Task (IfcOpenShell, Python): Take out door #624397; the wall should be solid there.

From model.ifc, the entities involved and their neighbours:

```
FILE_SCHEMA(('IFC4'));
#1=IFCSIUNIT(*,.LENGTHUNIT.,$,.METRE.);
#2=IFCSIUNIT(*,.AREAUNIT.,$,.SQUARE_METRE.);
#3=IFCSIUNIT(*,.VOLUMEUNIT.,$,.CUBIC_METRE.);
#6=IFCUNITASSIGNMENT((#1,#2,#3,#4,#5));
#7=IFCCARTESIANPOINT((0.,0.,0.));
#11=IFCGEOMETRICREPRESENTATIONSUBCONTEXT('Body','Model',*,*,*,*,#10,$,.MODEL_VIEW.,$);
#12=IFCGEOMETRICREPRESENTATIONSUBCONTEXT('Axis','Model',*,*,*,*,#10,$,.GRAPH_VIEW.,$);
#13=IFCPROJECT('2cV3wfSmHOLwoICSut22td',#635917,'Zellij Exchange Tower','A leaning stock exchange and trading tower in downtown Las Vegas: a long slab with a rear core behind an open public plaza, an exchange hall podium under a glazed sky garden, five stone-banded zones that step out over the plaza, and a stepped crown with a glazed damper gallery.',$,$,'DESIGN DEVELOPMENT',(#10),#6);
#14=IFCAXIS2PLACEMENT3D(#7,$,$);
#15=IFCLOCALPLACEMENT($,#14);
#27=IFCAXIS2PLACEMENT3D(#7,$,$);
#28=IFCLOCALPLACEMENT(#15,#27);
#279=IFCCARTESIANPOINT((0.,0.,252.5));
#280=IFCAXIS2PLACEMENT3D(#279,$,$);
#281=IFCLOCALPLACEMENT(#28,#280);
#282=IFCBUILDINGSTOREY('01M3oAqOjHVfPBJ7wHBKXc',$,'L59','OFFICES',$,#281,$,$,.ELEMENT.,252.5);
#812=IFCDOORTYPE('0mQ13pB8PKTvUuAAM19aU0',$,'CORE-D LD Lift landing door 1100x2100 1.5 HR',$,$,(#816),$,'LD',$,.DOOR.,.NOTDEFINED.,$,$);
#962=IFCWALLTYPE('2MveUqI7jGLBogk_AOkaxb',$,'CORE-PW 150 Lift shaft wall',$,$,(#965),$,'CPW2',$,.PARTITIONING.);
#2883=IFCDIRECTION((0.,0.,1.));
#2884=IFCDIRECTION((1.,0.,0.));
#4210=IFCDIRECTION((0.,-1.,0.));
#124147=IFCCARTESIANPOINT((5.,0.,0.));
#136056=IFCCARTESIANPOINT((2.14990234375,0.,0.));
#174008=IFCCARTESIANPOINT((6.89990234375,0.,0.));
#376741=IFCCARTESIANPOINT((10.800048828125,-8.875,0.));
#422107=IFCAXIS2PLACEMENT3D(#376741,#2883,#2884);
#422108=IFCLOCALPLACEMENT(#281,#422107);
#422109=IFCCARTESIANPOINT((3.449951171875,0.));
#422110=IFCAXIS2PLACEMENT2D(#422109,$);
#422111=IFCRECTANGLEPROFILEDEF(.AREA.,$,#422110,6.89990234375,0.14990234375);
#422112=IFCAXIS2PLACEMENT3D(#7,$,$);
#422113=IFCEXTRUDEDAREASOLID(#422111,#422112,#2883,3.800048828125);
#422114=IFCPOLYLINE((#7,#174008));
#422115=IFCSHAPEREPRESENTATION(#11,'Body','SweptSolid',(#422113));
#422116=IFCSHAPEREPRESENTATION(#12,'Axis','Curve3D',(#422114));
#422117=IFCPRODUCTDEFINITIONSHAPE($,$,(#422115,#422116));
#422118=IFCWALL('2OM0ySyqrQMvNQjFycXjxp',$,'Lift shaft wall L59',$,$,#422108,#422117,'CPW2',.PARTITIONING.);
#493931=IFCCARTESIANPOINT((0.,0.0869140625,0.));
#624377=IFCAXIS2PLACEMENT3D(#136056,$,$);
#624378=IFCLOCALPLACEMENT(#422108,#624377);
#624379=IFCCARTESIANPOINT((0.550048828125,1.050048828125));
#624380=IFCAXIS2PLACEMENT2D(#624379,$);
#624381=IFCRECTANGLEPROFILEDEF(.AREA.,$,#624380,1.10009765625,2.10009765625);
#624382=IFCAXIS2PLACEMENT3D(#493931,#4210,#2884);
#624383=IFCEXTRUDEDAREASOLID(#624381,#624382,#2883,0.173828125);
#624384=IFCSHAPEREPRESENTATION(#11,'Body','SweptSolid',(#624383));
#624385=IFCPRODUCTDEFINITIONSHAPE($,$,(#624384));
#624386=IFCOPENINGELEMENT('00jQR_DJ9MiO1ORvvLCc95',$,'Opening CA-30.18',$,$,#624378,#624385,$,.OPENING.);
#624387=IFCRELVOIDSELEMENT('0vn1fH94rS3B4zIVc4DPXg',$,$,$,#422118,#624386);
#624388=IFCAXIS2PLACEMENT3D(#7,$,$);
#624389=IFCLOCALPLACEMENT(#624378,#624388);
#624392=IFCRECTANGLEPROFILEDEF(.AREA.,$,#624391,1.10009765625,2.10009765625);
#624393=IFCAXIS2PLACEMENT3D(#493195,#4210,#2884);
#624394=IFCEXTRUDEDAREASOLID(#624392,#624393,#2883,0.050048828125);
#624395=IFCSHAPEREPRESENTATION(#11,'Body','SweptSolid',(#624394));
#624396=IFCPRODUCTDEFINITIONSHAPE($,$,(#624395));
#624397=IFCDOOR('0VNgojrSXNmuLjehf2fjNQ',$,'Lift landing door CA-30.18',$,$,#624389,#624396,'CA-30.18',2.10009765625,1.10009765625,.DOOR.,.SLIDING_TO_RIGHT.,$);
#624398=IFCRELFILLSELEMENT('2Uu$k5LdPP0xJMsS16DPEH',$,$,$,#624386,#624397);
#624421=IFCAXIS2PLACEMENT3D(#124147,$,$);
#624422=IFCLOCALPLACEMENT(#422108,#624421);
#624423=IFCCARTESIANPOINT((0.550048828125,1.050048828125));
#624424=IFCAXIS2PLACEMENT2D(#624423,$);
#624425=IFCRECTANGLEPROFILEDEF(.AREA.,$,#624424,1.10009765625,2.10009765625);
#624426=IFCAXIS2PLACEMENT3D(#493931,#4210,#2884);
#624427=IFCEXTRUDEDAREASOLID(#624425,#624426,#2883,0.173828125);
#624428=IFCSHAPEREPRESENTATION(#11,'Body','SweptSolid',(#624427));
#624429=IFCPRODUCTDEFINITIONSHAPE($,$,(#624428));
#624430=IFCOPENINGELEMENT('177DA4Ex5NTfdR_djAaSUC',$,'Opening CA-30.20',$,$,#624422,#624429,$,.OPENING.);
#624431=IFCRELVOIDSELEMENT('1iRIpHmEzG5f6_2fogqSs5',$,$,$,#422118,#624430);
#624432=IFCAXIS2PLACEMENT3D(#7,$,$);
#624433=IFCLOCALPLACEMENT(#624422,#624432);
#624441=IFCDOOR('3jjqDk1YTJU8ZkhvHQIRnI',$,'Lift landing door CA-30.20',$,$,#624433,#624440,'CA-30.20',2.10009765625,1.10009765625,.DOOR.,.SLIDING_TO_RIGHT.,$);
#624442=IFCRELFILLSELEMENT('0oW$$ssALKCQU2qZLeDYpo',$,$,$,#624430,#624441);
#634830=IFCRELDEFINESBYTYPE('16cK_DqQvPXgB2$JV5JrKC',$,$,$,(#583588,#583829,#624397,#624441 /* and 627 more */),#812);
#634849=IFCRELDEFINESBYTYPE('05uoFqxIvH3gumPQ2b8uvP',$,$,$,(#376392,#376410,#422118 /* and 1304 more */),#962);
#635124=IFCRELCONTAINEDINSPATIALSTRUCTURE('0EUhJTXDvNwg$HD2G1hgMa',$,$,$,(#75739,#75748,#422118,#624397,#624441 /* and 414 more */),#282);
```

```python
import ifcopenshell
import ifcopenshell.api.feature
import ifcopenshell.api.root
import ifcopenshell.geom
import ifcopenshell.util.shape

model = ifcopenshell.open("model.ifc")
settings = ifcopenshell.geom.settings()


def volume(element):
    """Net volume in cubic metres, openings subtracted."""
    shape = ifcopenshell.geom.create_shape(settings, element)
    return ifcopenshell.util.shape.get_volume(shape.geometry)


door = model.by_id(624397)
opening = door.FillsVoids[0].RelatingOpeningElement
wall = opening.VoidsElements[0].RelatingBuildingElement
before = volume(wall)

ifcopenshell.api.root.remove_product(model, product=door)
ifcopenshell.api.feature.remove_feature(model, feature=opening)

after = volume(wall)

print(f"wall volume {before:.3f} -> {after:.3f} m3")

model.write("model_rev.ifc")
```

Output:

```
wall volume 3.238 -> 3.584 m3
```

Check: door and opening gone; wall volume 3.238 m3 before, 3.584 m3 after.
